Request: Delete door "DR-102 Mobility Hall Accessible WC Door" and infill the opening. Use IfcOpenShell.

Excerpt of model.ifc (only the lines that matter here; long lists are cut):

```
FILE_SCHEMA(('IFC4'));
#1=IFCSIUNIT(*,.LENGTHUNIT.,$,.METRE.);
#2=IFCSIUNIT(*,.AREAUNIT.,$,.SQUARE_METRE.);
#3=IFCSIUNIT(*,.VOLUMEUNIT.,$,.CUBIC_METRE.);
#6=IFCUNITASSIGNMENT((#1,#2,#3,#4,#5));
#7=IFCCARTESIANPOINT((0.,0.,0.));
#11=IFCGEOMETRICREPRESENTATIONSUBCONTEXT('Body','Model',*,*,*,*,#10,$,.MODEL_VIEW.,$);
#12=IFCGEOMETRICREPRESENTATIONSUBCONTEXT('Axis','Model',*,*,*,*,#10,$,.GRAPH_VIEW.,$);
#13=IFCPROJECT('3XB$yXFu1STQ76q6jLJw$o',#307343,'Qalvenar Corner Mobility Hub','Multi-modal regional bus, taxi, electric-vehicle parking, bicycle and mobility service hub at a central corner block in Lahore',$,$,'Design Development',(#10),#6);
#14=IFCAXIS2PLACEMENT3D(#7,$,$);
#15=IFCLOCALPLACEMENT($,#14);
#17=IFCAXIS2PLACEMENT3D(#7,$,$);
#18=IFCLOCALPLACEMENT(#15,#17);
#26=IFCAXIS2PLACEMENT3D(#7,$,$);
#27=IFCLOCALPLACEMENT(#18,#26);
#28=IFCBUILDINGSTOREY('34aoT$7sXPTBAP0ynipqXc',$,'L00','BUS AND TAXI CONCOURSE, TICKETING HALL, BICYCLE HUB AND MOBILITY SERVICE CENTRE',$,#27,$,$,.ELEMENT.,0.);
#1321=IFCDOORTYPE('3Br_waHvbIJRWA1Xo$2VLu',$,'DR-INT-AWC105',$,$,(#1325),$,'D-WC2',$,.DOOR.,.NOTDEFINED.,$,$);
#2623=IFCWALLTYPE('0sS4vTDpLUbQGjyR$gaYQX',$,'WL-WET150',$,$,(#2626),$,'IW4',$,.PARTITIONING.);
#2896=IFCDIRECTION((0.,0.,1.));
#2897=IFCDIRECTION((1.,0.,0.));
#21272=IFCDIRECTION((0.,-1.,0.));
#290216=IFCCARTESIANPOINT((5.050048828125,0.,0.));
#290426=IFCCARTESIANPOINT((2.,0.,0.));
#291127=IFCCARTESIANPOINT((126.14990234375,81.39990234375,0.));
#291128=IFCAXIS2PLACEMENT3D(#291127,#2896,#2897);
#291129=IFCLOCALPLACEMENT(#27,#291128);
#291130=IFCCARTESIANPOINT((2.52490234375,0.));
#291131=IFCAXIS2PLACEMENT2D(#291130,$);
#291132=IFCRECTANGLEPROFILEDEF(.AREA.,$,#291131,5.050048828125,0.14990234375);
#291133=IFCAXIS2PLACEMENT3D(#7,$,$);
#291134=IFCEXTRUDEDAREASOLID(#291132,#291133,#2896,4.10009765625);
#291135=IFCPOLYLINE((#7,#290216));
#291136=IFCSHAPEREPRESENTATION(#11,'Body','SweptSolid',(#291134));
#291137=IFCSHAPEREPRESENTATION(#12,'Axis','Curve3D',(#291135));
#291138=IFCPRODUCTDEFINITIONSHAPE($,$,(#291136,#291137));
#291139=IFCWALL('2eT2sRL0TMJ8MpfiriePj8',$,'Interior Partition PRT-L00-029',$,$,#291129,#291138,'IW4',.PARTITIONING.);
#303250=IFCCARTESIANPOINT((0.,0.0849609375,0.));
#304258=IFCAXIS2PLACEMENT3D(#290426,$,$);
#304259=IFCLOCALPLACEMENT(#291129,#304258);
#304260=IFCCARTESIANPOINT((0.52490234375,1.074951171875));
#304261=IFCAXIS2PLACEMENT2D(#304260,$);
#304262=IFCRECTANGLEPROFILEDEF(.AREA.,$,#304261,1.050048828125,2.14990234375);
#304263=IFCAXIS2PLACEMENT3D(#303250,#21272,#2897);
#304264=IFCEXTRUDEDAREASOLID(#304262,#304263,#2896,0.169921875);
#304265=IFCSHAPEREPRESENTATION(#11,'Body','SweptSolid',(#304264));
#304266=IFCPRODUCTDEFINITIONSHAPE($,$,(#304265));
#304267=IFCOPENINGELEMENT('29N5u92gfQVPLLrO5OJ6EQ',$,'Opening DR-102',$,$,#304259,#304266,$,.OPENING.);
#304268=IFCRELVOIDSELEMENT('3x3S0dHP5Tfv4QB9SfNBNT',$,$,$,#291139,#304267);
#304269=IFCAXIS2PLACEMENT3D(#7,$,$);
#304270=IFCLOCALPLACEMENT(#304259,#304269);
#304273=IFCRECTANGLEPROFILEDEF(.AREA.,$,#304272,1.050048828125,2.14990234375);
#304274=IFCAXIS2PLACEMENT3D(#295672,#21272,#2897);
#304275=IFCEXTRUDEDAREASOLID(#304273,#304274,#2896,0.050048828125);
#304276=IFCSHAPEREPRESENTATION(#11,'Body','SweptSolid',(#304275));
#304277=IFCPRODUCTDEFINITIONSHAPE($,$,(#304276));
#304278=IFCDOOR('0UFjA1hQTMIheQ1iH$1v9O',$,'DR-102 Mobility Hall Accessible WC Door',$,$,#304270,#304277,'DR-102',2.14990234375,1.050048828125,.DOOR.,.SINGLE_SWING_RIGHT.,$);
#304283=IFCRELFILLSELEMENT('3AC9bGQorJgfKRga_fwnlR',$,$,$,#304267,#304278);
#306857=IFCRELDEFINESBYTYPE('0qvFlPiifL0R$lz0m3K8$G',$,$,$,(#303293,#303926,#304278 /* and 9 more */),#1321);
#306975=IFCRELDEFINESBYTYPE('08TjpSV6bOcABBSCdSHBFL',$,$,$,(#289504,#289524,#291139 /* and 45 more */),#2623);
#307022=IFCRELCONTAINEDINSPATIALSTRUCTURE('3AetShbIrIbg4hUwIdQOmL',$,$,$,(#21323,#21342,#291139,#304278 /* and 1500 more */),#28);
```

```python
import ifcopenshell
import ifcopenshell.api.feature
import ifcopenshell.api.root
import ifcopenshell.geom
import ifcopenshell.util.shape

model = ifcopenshell.open("model.ifc")
settings = ifcopenshell.geom.settings()


def volume(element):
    """Net volume in cubic metres, openings subtracted."""
    shape = ifcopenshell.geom.create_shape(settings, element)
    return ifcopenshell.util.shape.get_volume(shape.geometry)


door = model.by_guid("0UFjA1hQTMIheQ1iH$1v9O")
opening = door.FillsVoids[0].RelatingOpeningElement
wall = opening.VoidsElements[0].RelatingBuildingElement
before = volume(wall)

ifcopenshell.api.root.remove_product(model, product=door)
ifcopenshell.api.feature.remove_feature(model, feature=opening)

after = volume(wall)

print(f"wall volume {before:.3f} -> {after:.3f} m3")

model.write("model_updated.ifc")
```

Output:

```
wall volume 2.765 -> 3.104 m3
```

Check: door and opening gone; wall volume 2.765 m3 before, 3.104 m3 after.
